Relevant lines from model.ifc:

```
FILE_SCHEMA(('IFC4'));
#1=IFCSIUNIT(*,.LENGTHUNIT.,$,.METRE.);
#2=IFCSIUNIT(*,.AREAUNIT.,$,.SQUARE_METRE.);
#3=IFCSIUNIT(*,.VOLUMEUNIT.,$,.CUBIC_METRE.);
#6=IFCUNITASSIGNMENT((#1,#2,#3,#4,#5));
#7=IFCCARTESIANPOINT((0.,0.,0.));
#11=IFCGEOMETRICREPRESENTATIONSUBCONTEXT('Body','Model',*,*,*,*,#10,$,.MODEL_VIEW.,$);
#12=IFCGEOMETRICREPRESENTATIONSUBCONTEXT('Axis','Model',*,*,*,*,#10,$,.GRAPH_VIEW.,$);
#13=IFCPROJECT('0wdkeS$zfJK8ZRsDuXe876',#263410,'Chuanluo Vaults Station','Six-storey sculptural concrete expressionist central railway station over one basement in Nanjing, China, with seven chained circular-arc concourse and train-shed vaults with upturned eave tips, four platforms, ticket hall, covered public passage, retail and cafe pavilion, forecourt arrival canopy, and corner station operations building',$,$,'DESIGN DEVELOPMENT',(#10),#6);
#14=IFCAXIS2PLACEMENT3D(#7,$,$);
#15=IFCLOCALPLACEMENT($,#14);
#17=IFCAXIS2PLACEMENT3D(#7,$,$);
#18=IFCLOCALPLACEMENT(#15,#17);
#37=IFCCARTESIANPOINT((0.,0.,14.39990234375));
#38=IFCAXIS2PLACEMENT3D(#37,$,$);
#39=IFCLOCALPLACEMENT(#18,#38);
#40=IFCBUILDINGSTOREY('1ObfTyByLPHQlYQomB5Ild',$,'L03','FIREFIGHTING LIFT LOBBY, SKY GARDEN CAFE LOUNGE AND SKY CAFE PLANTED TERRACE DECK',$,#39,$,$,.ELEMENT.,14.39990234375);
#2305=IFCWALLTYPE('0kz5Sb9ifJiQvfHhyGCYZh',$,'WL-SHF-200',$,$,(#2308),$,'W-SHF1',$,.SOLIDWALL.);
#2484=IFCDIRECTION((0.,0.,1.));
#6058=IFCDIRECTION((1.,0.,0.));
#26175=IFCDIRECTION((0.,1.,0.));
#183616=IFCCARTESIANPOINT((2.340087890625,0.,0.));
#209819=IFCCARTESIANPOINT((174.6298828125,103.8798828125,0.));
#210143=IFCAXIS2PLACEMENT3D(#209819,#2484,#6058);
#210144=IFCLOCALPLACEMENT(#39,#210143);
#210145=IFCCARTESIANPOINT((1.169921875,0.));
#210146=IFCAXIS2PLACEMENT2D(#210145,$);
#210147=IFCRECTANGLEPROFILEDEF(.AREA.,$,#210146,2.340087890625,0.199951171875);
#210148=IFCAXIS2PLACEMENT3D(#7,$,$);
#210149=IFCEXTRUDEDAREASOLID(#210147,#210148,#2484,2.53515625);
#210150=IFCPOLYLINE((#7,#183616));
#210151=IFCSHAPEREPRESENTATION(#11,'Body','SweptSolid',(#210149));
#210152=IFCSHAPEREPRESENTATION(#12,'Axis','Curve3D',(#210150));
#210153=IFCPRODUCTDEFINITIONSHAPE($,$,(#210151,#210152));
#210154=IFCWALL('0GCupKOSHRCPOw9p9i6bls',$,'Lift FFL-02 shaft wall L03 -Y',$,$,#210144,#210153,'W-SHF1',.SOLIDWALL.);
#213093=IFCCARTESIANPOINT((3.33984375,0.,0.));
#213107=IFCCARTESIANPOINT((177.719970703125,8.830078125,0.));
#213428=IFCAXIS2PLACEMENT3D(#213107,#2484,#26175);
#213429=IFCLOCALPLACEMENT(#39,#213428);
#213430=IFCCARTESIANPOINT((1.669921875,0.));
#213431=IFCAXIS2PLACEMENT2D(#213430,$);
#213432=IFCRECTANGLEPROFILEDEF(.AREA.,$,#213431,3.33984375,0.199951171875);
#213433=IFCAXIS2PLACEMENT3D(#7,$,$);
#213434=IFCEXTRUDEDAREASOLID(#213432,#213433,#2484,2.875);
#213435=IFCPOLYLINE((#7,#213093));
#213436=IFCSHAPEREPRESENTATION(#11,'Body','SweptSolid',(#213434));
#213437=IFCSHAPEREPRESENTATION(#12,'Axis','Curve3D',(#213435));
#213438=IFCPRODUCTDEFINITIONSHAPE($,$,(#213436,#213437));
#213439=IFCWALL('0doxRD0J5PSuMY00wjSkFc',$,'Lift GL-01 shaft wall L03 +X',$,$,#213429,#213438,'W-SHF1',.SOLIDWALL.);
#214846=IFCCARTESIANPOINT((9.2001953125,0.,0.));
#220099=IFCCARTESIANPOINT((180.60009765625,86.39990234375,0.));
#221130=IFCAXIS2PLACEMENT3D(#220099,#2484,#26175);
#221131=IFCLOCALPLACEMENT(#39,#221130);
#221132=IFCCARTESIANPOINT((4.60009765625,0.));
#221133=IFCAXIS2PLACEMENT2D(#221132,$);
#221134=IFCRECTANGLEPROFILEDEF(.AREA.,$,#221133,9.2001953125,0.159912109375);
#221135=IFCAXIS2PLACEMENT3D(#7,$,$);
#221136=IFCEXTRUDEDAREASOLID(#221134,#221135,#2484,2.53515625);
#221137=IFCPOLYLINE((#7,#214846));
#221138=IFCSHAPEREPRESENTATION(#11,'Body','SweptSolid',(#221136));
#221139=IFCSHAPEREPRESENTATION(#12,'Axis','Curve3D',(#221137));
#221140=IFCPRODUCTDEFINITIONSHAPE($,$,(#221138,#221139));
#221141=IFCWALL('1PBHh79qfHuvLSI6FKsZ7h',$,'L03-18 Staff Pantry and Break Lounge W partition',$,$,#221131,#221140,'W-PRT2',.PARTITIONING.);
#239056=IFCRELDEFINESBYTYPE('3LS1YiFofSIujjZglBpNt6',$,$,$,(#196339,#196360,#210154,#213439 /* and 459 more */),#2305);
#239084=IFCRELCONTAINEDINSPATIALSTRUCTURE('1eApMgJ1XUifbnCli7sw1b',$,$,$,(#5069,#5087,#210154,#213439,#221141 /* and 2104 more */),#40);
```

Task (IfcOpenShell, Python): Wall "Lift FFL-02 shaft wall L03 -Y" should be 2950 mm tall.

```python
import ifcopenshell
import ifcopenshell.geom
import ifcopenshell.util.representation
import ifcopenshell.util.shape
import ifcopenshell.util.unit

model = ifcopenshell.open("model.ifc")
unit_scale = ifcopenshell.util.unit.calculate_unit_scale(model)
settings = ifcopenshell.geom.settings()


def volume(element):
    """Net volume in cubic metres, openings subtracted."""
    shape = ifcopenshell.geom.create_shape(settings, element)
    return ifcopenshell.util.shape.get_volume(shape.geometry)


wall = model.by_guid("0GCupKOSHRCPOw9p9i6bls")
before = volume(wall)

body = ifcopenshell.util.representation.get_representation(wall, "Model", "Body")
solid = body.Items[0]
old_height = solid.Depth
solid.Depth = 2.95 / unit_scale
after = volume(wall)

print(f"height {old_height:g} -> {solid.Depth:g}, volume {before:.3f} -> {after:.3f} m3")

model.write("model_edited.ifc")
```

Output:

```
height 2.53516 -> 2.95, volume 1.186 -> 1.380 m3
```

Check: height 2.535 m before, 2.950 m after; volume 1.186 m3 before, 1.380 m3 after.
